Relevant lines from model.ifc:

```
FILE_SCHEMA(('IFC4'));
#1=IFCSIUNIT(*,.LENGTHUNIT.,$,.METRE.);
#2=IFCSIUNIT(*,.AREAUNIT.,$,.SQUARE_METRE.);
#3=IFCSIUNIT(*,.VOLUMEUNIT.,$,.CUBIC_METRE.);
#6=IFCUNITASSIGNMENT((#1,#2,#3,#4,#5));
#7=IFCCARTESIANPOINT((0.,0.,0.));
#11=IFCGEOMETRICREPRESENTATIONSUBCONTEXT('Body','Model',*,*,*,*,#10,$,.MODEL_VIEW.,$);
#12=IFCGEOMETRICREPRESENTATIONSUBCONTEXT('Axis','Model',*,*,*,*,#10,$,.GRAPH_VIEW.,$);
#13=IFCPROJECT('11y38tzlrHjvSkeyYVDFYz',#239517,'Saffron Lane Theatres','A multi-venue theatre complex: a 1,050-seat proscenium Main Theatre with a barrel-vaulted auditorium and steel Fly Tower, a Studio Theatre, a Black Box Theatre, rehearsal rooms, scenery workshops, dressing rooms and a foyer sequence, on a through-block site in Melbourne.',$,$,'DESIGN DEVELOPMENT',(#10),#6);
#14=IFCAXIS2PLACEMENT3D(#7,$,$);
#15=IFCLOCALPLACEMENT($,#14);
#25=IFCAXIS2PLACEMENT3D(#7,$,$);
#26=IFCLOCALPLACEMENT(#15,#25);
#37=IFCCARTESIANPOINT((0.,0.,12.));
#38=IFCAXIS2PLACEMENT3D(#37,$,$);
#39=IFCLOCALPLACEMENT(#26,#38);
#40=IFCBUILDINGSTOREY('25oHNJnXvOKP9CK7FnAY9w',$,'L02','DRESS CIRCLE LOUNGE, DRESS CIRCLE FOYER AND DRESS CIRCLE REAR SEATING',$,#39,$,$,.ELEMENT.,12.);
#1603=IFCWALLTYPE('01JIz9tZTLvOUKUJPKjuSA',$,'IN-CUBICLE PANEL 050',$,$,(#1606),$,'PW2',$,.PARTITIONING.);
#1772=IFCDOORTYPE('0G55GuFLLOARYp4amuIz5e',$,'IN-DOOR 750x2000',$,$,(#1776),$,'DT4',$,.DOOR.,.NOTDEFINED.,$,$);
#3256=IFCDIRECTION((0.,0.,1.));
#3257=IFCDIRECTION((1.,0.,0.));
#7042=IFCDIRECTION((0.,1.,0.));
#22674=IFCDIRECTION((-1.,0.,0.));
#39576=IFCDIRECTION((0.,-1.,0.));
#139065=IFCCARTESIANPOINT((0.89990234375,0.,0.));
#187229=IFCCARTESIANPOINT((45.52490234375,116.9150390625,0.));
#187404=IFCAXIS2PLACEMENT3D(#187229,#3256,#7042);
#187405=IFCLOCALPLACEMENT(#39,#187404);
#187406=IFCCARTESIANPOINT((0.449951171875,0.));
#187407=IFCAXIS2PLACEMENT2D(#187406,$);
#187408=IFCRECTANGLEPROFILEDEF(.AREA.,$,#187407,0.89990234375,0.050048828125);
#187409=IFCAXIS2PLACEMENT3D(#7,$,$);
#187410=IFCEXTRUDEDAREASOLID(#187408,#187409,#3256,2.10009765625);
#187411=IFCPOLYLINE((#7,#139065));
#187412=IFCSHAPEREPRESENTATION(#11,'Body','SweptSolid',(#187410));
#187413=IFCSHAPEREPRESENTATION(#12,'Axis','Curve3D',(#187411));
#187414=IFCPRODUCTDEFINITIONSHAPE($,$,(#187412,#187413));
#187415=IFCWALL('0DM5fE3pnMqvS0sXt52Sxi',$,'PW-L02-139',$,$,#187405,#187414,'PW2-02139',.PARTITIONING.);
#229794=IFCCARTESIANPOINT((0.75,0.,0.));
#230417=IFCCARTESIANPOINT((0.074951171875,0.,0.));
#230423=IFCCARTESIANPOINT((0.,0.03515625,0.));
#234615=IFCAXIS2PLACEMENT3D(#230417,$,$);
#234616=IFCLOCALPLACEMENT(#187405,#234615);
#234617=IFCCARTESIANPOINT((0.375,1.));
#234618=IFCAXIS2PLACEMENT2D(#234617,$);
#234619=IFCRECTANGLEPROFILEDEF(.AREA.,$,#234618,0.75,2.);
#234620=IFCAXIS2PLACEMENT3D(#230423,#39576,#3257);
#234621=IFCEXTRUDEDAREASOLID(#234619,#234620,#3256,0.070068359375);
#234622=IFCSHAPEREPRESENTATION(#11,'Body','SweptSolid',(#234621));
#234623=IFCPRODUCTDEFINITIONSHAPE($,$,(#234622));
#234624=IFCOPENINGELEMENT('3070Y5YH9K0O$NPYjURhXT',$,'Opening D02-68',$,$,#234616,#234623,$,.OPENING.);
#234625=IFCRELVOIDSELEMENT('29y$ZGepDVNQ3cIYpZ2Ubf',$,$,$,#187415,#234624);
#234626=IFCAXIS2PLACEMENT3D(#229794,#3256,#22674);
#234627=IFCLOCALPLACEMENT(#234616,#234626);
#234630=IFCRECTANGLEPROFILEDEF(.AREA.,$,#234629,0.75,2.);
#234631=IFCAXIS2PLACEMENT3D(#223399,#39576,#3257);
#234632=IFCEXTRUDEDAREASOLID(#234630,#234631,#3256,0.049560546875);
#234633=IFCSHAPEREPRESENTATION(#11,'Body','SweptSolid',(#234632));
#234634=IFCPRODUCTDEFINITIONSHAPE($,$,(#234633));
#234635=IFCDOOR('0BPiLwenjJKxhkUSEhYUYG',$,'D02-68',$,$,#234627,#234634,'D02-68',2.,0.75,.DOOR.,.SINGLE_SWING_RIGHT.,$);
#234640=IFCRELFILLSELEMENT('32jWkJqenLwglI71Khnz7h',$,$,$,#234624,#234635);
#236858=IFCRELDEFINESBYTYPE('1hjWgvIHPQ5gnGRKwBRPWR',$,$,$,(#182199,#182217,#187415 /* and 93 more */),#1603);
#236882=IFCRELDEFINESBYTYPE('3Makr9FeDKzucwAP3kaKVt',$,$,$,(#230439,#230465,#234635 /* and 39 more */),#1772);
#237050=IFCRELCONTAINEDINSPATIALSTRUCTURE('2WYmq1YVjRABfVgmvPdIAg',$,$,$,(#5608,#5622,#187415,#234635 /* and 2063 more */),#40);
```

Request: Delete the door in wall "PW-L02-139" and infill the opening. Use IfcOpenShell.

```python
import ifcopenshell
import ifcopenshell.api.feature
import ifcopenshell.api.root
import ifcopenshell.geom
import ifcopenshell.util.shape

model = ifcopenshell.open("model.ifc")
settings = ifcopenshell.geom.settings()


def volume(element):
    """Net volume in cubic metres, openings subtracted."""
    shape = ifcopenshell.geom.create_shape(settings, element)
    return ifcopenshell.util.shape.get_volume(shape.geometry)


door = model.by_id(234635)
opening = door.FillsVoids[0].RelatingOpeningElement
wall = opening.VoidsElements[0].RelatingBuildingElement
before = volume(wall)

ifcopenshell.api.root.remove_product(model, product=door)
ifcopenshell.api.feature.remove_feature(model, feature=opening)

after = volume(wall)

print(f"wall volume {before:.3f} -> {after:.3f} m3")

model.write("model_updated.ifc")
```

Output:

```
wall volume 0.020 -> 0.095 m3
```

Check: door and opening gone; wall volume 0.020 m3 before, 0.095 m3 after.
